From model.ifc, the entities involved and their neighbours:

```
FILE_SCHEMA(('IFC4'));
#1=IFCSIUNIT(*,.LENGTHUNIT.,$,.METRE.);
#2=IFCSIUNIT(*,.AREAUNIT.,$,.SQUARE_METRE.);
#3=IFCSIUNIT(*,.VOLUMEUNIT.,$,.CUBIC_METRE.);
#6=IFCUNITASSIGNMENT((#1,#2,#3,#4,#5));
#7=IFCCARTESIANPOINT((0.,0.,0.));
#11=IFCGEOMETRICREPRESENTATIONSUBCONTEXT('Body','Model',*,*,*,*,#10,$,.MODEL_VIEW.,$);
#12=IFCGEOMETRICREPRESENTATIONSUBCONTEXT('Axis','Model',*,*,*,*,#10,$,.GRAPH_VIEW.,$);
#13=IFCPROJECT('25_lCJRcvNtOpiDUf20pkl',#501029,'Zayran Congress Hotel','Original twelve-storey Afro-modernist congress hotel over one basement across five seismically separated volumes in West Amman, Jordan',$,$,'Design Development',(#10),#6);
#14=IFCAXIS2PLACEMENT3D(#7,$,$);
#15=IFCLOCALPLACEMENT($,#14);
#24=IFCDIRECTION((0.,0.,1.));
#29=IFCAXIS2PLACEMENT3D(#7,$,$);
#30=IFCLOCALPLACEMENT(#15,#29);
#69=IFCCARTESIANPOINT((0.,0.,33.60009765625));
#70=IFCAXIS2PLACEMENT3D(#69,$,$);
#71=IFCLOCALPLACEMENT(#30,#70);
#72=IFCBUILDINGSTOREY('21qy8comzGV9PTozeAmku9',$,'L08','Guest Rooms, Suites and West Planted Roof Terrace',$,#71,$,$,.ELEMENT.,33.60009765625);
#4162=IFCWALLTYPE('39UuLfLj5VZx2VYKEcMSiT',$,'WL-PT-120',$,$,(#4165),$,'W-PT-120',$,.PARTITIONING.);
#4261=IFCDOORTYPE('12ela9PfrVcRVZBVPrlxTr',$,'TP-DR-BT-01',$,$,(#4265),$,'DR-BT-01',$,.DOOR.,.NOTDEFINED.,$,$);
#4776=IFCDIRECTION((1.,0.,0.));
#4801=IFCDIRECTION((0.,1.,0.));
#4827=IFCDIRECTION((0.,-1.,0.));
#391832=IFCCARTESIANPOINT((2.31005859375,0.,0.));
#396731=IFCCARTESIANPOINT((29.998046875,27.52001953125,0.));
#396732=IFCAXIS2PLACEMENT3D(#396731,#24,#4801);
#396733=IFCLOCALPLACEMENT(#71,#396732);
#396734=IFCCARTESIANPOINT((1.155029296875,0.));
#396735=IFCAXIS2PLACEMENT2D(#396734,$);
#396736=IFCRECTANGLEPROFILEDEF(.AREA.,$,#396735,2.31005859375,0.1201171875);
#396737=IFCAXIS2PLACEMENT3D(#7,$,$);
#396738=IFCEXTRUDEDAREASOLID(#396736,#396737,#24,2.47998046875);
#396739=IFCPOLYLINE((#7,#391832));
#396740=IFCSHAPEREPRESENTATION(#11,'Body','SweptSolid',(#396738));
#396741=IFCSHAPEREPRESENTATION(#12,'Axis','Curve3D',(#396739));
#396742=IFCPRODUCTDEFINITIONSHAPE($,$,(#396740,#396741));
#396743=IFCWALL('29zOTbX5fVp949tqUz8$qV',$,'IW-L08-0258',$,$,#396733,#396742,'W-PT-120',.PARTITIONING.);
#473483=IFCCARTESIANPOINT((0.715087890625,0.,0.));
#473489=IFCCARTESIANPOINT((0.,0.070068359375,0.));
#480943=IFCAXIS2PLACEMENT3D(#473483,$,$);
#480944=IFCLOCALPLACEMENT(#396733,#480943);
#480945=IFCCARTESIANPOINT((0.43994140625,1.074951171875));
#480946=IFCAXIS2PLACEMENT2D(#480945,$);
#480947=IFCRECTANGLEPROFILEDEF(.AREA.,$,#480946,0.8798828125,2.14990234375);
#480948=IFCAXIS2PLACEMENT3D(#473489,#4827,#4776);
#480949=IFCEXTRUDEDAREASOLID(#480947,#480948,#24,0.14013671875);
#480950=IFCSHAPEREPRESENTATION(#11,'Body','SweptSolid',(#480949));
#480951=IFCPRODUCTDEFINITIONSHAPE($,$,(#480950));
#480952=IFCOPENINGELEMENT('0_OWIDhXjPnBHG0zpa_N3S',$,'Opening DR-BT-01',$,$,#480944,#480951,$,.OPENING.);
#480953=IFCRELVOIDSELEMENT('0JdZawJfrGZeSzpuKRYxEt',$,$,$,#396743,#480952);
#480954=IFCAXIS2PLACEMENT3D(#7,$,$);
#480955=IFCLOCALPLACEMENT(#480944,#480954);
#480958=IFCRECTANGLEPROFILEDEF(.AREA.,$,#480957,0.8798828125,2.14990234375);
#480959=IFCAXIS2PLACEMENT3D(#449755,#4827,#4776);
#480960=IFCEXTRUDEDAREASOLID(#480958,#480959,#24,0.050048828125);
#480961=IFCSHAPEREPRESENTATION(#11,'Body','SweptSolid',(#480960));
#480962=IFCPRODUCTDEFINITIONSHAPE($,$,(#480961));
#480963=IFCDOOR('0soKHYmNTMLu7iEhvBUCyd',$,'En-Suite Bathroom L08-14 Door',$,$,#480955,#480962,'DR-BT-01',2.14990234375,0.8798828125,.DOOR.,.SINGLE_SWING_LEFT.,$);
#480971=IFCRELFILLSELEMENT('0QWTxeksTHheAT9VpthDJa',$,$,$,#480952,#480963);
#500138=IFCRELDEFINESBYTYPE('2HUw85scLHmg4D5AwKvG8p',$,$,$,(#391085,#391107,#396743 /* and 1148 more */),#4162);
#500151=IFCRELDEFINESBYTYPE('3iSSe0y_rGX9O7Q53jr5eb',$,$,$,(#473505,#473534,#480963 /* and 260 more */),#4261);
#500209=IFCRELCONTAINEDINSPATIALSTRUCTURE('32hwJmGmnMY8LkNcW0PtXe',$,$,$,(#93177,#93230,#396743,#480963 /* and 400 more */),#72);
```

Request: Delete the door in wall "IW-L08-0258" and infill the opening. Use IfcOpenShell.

```python
import ifcopenshell
import ifcopenshell.api.feature
import ifcopenshell.api.root
import ifcopenshell.geom
import ifcopenshell.util.shape

model = ifcopenshell.open("model.ifc")
settings = ifcopenshell.geom.settings()


def volume(element):
    """Net volume in cubic metres, openings subtracted."""
    shape = ifcopenshell.geom.create_shape(settings, element)
    return ifcopenshell.util.shape.get_volume(shape.geometry)


door = model.by_guid("0soKHYmNTMLu7iEhvBUCyd")
opening = door.FillsVoids[0].RelatingOpeningElement
wall = opening.VoidsElements[0].RelatingBuildingElement
before = volume(wall)

ifcopenshell.api.root.remove_product(model, product=door)
ifcopenshell.api.feature.remove_feature(model, feature=opening)

after = volume(wall)

print(f"wall volume {before:.3f} -> {after:.3f} m3")

model.write("model-out.ifc")
```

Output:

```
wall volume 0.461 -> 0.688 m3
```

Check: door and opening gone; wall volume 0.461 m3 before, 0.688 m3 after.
